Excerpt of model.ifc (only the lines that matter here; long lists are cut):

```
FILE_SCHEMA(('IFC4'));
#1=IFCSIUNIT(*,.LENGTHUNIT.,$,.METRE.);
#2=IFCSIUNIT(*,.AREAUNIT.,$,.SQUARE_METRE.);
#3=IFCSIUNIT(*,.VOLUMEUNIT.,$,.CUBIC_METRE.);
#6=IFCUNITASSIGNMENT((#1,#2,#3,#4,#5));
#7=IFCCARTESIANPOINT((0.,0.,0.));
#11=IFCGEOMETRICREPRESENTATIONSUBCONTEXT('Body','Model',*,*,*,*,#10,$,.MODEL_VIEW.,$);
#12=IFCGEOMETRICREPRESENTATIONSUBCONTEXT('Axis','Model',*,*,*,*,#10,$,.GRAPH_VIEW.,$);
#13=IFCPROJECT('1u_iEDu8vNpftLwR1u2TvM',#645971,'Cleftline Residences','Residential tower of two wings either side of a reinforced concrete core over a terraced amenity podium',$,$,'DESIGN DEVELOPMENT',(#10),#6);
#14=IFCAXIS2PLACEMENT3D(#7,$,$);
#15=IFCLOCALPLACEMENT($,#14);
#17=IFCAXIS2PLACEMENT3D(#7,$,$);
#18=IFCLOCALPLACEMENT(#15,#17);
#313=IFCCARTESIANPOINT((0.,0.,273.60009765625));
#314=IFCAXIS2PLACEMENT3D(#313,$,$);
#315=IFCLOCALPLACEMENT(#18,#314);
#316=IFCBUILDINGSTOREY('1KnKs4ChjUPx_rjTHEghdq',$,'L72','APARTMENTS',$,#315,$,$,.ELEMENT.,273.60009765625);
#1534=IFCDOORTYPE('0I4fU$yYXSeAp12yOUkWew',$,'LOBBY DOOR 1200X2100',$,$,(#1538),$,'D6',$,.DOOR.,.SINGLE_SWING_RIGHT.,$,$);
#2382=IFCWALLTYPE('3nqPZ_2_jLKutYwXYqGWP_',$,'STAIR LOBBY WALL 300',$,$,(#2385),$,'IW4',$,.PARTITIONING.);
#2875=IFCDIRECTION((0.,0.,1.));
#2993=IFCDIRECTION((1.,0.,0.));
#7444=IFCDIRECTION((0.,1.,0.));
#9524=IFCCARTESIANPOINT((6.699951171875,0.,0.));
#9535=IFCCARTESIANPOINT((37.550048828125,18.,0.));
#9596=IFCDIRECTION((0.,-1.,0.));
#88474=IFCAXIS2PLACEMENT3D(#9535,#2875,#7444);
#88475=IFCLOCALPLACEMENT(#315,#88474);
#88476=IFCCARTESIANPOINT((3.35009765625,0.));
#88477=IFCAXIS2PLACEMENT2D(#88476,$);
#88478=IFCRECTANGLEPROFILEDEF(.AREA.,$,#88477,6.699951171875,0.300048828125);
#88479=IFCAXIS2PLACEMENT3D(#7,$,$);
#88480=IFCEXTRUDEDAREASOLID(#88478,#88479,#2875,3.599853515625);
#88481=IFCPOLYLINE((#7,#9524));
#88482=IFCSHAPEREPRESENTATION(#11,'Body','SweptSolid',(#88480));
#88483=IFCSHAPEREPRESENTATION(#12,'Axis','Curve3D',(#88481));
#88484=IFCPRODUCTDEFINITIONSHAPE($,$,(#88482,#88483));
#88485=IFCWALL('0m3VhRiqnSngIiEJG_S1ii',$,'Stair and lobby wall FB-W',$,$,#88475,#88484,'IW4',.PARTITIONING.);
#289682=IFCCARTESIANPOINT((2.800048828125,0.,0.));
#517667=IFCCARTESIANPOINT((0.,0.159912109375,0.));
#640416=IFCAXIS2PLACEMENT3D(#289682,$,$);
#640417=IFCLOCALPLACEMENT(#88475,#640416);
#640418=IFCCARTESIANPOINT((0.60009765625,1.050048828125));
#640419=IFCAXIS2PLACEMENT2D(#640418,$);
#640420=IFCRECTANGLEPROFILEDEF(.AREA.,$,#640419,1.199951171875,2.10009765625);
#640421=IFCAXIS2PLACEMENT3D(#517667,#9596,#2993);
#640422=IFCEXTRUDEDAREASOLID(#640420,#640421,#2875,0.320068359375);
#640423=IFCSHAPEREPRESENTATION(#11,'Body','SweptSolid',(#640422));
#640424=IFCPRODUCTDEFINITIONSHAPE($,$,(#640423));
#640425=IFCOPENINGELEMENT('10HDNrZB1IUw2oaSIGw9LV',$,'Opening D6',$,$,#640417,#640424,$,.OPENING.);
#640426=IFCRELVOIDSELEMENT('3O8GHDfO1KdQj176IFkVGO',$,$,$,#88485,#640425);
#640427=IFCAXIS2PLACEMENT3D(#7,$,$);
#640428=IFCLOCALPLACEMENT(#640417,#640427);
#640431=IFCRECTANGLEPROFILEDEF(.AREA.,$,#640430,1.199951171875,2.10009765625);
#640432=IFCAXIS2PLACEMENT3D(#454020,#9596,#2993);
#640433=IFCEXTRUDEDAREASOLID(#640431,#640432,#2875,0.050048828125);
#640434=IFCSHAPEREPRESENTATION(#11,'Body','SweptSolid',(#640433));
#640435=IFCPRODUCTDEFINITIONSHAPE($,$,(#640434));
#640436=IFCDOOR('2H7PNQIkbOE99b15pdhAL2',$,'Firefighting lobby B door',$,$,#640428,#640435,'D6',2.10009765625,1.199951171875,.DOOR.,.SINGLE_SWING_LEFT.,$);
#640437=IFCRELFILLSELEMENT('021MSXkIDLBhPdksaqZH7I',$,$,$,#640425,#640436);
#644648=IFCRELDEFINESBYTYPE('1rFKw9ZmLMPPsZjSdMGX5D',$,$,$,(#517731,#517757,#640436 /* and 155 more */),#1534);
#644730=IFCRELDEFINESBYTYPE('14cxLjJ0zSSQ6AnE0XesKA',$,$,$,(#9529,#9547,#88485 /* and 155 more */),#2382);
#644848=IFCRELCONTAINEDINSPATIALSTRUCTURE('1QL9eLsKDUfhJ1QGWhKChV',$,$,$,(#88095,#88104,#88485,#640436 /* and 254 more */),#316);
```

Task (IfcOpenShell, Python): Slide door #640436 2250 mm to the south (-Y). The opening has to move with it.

```python
import ifcopenshell
import ifcopenshell.api.geometry
import ifcopenshell.util.placement

model = ifcopenshell.open("model.ifc")

door = model.by_guid("2H7PNQIkbOE99b15pdhAL2")
opening = door.FillsVoids[0].RelatingOpeningElement
wall = opening.VoidsElements[0].RelatingBuildingElement

wall_matrix = ifcopenshell.util.placement.get_local_placement(wall.ObjectPlacement)
shift = wall_matrix[:3, 0] * -2.25
before = ifcopenshell.util.placement.get_local_placement(door.ObjectPlacement)[:3, 3].copy()

# The door is placed relative to its opening, so it follows when the opening moves.
matrix = ifcopenshell.util.placement.get_local_placement(opening.ObjectPlacement)
matrix[:3, 3] += shift
ifcopenshell.api.geometry.edit_object_placement(
    model, product=opening, matrix=matrix, is_si=False, should_transform_children=True
)

after = ifcopenshell.util.placement.get_local_placement(door.ObjectPlacement)[:3, 3]
print("door moved by", (after - before).round(3) + 0.0)

model.write("model_edited.ifc")
```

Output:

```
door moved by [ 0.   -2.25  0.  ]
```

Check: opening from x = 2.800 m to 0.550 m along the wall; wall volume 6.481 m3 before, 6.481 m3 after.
